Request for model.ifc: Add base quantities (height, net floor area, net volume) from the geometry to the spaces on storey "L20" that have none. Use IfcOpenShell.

First a look at what the model holds.

```python
import ifcopenshell
import ifcopenshell.util.element
import ifcopenshell.util.unit

model = ifcopenshell.open("model.ifc")
print(model.schema)
for unit_type in ("LENGTHUNIT", "AREAUNIT", "VOLUMEUNIT"):
    print(unit_type, ifcopenshell.util.unit.calculate_unit_scale(model, unit_type))
storey = next(s for s in model.by_type("IfcBuildingStorey") if s.Name == "L20")
spaces = [e for e in ifcopenshell.util.element.get_decomposition(storey) if e.is_a("IfcSpace")]
for e in sorted(spaces, key=lambda e: e.id()):
    print(e.id(), e.is_a(), e.Name, list(ifcopenshell.util.element.get_psets(e, qtos_only=True)), sep=" | ")
```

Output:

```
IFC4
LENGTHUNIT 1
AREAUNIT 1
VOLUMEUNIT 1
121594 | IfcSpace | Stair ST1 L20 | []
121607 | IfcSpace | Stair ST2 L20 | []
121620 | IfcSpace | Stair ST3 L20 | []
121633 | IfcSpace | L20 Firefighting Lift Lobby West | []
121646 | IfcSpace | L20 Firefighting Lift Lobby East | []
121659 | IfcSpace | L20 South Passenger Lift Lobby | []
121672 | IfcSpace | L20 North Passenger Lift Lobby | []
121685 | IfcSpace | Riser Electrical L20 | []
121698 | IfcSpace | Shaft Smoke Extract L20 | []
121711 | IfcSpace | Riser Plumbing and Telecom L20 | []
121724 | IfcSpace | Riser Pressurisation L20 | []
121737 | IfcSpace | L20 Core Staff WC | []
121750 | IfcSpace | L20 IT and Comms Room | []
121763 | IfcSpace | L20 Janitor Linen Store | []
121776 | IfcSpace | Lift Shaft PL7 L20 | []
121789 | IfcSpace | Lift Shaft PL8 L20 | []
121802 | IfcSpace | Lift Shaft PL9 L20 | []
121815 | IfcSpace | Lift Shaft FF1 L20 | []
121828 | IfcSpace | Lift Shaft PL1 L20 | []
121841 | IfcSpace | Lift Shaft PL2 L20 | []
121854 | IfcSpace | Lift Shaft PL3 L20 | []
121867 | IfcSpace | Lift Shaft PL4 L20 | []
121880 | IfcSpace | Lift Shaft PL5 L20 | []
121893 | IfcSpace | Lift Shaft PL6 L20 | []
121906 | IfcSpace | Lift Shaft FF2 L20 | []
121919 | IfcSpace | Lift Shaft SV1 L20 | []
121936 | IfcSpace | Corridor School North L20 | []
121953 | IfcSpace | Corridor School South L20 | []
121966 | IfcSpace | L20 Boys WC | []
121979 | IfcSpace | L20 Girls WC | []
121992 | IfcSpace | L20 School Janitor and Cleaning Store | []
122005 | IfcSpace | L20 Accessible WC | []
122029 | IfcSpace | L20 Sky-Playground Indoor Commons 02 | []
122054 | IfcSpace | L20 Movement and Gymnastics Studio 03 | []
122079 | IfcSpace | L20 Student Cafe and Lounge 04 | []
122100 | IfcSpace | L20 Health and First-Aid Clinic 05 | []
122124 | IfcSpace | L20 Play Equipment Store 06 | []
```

```python
import ifcopenshell
import ifcopenshell.api.pset
import ifcopenshell.geom
import ifcopenshell.util.element
import ifcopenshell.util.shape
import ifcopenshell.util.unit

model = ifcopenshell.open("model.ifc")
unit_scale = ifcopenshell.util.unit.calculate_unit_scale(model)
area_scale = ifcopenshell.util.unit.calculate_unit_scale(model, "AREAUNIT")
volume_scale = ifcopenshell.util.unit.calculate_unit_scale(model, "VOLUMEUNIT")
settings = ifcopenshell.geom.settings()

storey = next(s for s in model.by_type("IfcBuildingStorey") if s.Name == "L20")
spaces = [e for e in ifcopenshell.util.element.get_decomposition(storey) if e.is_a("IfcSpace")]

for e in sorted(spaces, key=lambda e: e.id()):
    if ifcopenshell.util.element.get_psets(e, qtos_only=True, should_inherit=False):
        continue
    # Geometry comes back in metres, in the element's own axes.
    shape = ifcopenshell.geom.create_shape(settings, e)
    values = {
        "Height": ifcopenshell.util.shape.get_z(shape.geometry) / unit_scale,
        "NetFloorArea": ifcopenshell.util.shape.get_footprint_area(shape.geometry) / area_scale,
        "NetVolume": ifcopenshell.util.shape.get_volume(shape.geometry) / volume_scale,
    }
    qto = ifcopenshell.api.pset.add_qto(model, product=e, name="Qto_SpaceBaseQuantities")
    ifcopenshell.api.pset.edit_qto(model, qto=qto, properties=values)
    print(e.id(), {k: round(v, 3) for k, v in values.items()})

model.write("model_rev.ifc")
```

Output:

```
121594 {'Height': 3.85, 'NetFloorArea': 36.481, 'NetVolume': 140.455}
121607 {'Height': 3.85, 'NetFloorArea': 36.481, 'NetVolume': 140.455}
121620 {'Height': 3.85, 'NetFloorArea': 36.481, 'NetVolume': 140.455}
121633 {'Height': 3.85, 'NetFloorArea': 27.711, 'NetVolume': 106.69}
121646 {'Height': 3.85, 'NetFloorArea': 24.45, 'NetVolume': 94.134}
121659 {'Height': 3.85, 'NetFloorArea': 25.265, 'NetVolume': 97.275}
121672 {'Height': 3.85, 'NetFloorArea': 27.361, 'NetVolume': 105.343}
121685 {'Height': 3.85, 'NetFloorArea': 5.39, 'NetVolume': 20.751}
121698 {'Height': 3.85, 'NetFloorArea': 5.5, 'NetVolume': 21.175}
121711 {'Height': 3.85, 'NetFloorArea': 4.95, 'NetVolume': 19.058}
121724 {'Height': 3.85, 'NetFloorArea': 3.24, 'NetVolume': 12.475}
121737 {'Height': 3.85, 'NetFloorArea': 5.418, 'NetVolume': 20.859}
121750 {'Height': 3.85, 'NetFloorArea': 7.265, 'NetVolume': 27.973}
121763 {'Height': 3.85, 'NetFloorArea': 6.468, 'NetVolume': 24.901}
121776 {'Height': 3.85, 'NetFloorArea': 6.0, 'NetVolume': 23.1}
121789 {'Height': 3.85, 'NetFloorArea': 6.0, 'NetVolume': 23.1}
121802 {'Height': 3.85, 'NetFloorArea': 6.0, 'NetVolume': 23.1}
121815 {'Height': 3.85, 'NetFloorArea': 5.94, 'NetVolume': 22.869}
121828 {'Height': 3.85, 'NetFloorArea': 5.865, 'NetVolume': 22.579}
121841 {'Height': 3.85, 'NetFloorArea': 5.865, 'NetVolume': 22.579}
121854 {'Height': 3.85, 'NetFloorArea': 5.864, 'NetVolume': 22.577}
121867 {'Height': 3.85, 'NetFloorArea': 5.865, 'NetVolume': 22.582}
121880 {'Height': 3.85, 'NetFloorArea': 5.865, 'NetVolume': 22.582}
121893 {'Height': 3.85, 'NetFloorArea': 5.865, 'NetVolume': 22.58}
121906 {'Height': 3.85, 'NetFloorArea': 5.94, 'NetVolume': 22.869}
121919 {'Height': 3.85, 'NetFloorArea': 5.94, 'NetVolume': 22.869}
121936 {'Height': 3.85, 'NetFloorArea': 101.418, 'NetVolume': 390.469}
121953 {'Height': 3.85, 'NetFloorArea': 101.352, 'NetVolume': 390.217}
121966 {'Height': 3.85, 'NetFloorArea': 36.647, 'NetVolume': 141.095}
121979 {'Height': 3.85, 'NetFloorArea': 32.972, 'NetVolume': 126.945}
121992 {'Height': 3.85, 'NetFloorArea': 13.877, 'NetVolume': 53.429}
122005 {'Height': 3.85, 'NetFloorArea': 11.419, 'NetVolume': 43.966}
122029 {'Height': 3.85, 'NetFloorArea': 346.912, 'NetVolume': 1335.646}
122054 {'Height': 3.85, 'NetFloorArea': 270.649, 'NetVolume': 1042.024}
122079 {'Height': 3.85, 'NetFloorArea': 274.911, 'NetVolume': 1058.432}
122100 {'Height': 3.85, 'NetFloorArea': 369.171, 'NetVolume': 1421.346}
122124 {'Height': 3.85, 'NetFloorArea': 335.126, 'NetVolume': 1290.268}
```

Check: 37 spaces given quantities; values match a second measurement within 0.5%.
